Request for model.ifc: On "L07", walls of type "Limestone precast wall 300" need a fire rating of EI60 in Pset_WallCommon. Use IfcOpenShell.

First a look at what the model holds.

```python
import ifcopenshell
import ifcopenshell.util.element

model = ifcopenshell.open("model.ifc")
print(model.schema)
storey = next(s for s in model.by_type("IfcBuildingStorey") if s.Name == "L07")
walls = [e for e in ifcopenshell.util.element.get_decomposition(storey) if e.is_a("IfcWall")]
seen = {}
for e in walls:
    element_type = ifcopenshell.util.element.get_type(e)
    key = (element_type.Name if element_type != e and element_type else None, ifcopenshell.util.element.get_pset(e, "Pset_WallCommon", "FireRating"))
    seen[key] = seen.get(key, 0) + 1
for (name, value), count in sorted(seen.items(), key=str):
    print(count, "x", name, "|", value)
```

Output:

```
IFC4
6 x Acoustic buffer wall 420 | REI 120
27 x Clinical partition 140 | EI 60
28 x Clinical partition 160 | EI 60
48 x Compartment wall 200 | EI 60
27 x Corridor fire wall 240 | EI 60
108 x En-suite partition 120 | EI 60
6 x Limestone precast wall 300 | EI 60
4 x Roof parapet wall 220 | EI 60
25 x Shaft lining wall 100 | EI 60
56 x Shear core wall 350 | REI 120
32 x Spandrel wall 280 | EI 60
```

```python
import ifcopenshell
import ifcopenshell.api.pset
import ifcopenshell.util.element

model = ifcopenshell.open("model.ifc")

storey = next(s for s in model.by_type("IfcBuildingStorey") if s.Name == "L07")
walls = [e for e in ifcopenshell.util.element.get_decomposition(storey) if e.is_a("IfcWall")]

count = 0
for e in walls:
    element_type = ifcopenshell.util.element.get_type(e)
    if element_type in (None, e) or element_type.Name != "Limestone precast wall 300":
        continue
    # add_pset returns the element's existing set when there is one.
    pset = ifcopenshell.api.pset.add_pset(model, product=e, name="Pset_WallCommon")
    ifcopenshell.api.pset.edit_pset(model, pset=pset, properties={"FireRating": "EI60"})
    count += 1

print(count, "walls updated")

model.write("model_edited.ifc")
```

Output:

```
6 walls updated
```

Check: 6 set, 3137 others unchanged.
